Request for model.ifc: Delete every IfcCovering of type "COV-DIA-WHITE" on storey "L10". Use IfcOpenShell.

First a look at what the model holds.

```python
import ifcopenshell
import ifcopenshell.util.element

model = ifcopenshell.open("model.ifc")
print(model.schema)
storey = next(s for s in model.by_type("IfcBuildingStorey") if s.Name == "L10")
coverings = [e for e in ifcopenshell.util.element.get_decomposition(storey) if e.is_a("IfcCovering")]
seen = {}
for e in coverings:
    element_type = ifcopenshell.util.element.get_type(e)
    name = element_type.Name if element_type not in (None, e) else None
    seen[name] = seen.get(name, 0) + 1
for name, count in sorted(seen.items(), key=str):
    print(count, "x", name)
```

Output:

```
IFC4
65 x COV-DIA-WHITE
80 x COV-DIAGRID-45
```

```python
import ifcopenshell
import ifcopenshell.api.root
import ifcopenshell.util.element

model = ifcopenshell.open("model.ifc")

storey = next(s for s in model.by_type("IfcBuildingStorey") if s.Name == "L10")
coverings = [e for e in ifcopenshell.util.element.get_decomposition(storey) if e.is_a("IfcCovering")]
targets = [e for e in coverings if (t := ifcopenshell.util.element.get_type(e)) not in (None, e) and t.Name == "COV-DIA-WHITE"]

for e in targets:
    ifcopenshell.api.root.remove_product(model, product=e)
print(len(targets), "removed")

model.write("model_v2.ifc")
```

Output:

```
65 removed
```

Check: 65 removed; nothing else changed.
